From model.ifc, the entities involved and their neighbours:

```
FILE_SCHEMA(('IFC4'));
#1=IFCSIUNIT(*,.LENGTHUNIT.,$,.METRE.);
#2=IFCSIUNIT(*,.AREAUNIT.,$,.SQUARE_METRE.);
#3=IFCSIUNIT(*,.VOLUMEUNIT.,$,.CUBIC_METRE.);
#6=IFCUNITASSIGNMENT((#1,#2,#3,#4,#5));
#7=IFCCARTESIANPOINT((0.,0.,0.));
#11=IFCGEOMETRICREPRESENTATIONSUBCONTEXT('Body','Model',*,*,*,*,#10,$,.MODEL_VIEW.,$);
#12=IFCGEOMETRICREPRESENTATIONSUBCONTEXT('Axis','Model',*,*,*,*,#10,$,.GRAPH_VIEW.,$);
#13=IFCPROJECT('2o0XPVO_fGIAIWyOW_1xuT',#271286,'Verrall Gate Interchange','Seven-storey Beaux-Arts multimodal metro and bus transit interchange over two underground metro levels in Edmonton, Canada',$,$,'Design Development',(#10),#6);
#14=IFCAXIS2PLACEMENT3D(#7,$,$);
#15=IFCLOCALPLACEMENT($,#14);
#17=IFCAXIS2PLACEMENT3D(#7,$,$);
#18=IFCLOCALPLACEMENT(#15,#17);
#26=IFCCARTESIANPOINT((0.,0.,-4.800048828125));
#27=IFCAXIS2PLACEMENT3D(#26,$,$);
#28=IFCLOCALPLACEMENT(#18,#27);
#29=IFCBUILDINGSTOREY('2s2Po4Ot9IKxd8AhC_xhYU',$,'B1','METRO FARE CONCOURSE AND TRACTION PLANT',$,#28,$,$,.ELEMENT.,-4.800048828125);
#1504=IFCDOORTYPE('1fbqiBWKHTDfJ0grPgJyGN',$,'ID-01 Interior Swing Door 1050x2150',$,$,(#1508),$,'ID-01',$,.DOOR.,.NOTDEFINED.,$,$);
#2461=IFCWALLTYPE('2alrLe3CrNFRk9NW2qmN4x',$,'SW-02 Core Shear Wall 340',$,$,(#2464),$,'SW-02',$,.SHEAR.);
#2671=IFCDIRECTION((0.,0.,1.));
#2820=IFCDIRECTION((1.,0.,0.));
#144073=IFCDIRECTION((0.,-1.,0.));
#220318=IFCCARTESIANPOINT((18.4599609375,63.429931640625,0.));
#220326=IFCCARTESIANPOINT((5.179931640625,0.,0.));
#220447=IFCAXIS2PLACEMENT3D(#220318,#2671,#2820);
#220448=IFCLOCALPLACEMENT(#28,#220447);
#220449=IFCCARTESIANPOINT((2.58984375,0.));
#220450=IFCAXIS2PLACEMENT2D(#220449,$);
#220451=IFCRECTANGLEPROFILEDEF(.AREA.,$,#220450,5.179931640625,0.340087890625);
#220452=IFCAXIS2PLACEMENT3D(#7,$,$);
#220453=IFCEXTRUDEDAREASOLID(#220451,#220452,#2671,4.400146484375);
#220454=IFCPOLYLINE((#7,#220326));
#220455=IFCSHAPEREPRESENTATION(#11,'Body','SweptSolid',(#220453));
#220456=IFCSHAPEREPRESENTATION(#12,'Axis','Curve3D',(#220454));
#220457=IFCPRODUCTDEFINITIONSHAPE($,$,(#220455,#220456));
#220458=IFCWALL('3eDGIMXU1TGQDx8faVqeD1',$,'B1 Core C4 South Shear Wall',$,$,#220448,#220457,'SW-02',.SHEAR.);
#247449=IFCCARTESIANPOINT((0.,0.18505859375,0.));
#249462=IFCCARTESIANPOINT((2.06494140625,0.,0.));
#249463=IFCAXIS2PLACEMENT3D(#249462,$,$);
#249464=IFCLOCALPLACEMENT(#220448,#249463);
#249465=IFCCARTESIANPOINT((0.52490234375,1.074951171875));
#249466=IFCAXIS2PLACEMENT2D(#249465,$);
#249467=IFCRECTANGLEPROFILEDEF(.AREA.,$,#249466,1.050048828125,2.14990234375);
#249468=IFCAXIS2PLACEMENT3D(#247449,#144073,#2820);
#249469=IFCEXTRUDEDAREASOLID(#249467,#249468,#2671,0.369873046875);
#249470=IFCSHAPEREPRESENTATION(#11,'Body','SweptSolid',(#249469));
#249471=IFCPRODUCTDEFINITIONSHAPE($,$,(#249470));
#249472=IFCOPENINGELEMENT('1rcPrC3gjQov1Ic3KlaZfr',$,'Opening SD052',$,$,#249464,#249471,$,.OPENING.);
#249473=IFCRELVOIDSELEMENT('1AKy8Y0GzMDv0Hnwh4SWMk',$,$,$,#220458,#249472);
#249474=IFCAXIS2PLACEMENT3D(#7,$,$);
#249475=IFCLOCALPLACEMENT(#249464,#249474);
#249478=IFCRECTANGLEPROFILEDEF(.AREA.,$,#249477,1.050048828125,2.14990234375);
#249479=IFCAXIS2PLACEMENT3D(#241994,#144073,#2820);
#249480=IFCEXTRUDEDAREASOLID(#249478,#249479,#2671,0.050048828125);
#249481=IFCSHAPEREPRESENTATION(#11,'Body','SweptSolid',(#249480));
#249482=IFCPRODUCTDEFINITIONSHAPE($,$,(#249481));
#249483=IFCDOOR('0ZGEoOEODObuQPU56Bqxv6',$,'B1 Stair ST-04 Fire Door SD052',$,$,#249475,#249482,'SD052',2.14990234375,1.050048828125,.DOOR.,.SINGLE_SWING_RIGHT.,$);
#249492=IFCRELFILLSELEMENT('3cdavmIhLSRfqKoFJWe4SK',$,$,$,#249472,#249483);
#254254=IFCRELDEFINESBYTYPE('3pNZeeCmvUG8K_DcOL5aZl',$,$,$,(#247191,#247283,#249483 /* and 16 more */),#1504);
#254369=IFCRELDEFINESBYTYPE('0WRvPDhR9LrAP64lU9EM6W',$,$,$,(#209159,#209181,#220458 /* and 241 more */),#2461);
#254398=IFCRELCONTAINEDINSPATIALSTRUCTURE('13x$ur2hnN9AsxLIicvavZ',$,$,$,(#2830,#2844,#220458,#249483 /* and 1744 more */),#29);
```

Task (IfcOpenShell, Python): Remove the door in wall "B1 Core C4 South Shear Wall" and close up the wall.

```python
import ifcopenshell
import ifcopenshell.api.feature
import ifcopenshell.api.root
import ifcopenshell.geom
import ifcopenshell.util.shape

model = ifcopenshell.open("model.ifc")
settings = ifcopenshell.geom.settings()


def volume(element):
    """Net volume in cubic metres, openings subtracted."""
    shape = ifcopenshell.geom.create_shape(settings, element)
    return ifcopenshell.util.shape.get_volume(shape.geometry)


door = model.by_id(249483)
opening = door.FillsVoids[0].RelatingOpeningElement
wall = opening.VoidsElements[0].RelatingBuildingElement
before = volume(wall)

ifcopenshell.api.root.remove_product(model, product=door)
ifcopenshell.api.feature.remove_feature(model, feature=opening)

after = volume(wall)

print(f"wall volume {before:.3f} -> {after:.3f} m3")

model.write("model_v2.ifc")
```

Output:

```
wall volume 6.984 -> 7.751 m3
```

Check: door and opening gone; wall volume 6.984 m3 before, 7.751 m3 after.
